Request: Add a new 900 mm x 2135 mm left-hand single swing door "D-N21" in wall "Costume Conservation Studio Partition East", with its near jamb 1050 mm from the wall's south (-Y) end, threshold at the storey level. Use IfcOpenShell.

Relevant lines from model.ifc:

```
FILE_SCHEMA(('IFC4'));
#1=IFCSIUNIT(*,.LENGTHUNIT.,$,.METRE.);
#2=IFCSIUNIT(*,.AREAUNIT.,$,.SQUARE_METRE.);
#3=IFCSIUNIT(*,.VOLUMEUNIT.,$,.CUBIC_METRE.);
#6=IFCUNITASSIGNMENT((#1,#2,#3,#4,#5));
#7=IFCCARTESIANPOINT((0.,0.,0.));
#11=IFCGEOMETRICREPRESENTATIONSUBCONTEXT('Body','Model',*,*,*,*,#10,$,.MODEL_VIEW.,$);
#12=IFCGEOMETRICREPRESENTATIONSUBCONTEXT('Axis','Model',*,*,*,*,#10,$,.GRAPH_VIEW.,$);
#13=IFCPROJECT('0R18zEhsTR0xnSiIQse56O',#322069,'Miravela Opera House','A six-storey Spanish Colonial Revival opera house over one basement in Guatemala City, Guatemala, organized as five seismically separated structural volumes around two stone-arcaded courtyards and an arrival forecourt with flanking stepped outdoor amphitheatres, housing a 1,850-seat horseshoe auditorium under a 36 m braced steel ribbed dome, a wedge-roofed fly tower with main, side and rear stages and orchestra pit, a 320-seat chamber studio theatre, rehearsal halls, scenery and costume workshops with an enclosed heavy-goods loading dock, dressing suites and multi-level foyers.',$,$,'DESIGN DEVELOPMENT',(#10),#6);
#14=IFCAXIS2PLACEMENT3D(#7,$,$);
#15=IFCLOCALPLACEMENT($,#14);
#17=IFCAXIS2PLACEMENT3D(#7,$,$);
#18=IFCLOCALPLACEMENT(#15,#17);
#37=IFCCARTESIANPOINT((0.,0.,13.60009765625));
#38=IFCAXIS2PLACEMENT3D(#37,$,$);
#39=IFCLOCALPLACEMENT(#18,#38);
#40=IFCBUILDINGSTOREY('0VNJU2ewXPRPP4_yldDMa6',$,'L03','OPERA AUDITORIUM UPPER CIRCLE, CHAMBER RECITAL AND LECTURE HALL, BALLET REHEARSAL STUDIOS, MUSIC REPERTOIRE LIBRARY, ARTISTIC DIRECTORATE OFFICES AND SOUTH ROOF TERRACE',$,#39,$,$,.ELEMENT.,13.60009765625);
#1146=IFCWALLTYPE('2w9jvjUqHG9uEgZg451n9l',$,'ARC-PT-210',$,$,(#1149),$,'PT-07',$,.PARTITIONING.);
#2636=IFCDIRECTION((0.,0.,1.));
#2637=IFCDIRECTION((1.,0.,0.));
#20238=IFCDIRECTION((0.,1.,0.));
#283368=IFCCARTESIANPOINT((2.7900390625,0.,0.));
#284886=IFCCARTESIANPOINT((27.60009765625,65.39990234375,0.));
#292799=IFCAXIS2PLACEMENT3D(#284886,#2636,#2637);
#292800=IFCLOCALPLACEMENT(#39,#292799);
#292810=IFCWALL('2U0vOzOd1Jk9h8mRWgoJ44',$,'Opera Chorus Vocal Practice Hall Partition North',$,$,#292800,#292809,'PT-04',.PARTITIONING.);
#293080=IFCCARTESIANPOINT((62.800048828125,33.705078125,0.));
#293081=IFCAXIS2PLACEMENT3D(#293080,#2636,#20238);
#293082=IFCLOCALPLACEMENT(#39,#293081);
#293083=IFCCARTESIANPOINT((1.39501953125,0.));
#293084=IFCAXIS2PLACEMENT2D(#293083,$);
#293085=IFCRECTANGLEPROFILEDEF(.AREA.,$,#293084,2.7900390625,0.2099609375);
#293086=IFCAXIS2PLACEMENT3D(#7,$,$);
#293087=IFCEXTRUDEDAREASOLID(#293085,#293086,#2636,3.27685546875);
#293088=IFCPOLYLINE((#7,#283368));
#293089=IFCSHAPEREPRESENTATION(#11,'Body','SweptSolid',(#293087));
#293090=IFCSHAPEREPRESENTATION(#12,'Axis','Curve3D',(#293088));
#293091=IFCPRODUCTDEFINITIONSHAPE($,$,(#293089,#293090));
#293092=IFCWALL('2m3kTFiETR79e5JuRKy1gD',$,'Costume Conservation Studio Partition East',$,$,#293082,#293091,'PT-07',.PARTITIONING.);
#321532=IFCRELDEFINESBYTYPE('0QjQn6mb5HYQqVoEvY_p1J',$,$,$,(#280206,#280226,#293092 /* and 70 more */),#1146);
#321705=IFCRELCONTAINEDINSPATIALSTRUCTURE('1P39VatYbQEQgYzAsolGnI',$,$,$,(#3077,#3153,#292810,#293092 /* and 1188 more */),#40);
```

```python
import numpy as np
import ifcopenshell
import ifcopenshell.api.feature
import ifcopenshell.api.geometry
import ifcopenshell.api.root
import ifcopenshell.api.spatial
import ifcopenshell.geom
import ifcopenshell.util.element
import ifcopenshell.util.placement
import ifcopenshell.util.representation
import ifcopenshell.util.shape
import ifcopenshell.util.unit

model = ifcopenshell.open("model.ifc")
unit_scale = ifcopenshell.util.unit.calculate_unit_scale(model)
settings = ifcopenshell.geom.settings()


def volume(element):
    """Net volume in cubic metres, openings subtracted."""
    shape = ifcopenshell.geom.create_shape(settings, element)
    return ifcopenshell.util.shape.get_volume(shape.geometry)


wall = model.by_guid("2m3kTFiETR79e5JuRKy1gD")
storey = ifcopenshell.util.element.get_container(wall, ifc_class="IfcBuildingStorey")
context = ifcopenshell.util.representation.get_context(model, "Model", "Body", "MODEL_VIEW")
before = volume(wall)

width, height, from_end, sill = 0.9, 2.135, 1.05, 0.0  # metres

# The wall runs along its own X axis, and the end named is its -X end.
wall_shape = ifcopenshell.geom.create_shape(settings, wall)
x, y, z = ifcopenshell.util.shape.get_vertices(wall_shape.geometry).T
start = x.min() + from_end
face, thickness = float(y.min()), float(y.max() - y.min())
wall_matrix = ifcopenshell.util.placement.get_local_placement(wall.ObjectPlacement)
level = ifcopenshell.util.placement.get_local_placement(storey.ObjectPlacement)[2, 3]


def in_wall(x, y):
    """Placement at x, y metres in the wall's axes, at sill height."""
    matrix = wall_matrix.copy()
    matrix[:, 3] = wall_matrix @ np.array([x / unit_scale, y / unit_scale, 0.0, 1.0])
    matrix[2, 3] = level + sill / unit_scale
    return matrix


# Opening: a box that overshoots both wall faces by 50 mm.
opening = ifcopenshell.api.root.create_entity(model, ifc_class="IfcOpeningElement", predefined_type="OPENING")
box = ifcopenshell.api.geometry.add_wall_representation(
    model, context=context, length=width, height=height, thickness=thickness + 0.1
)
ifcopenshell.api.geometry.assign_representation(model, product=opening, representation=box)
ifcopenshell.api.geometry.edit_object_placement(model, product=opening, matrix=in_wall(start, face - 0.05), is_si=False)
ifcopenshell.api.feature.add_feature(model, feature=opening, element=wall)

door = ifcopenshell.api.root.create_entity(model, ifc_class="IfcDoor", name="D-N21", predefined_type="DOOR")
door.OverallWidth, door.OverallHeight = width / unit_scale, height / unit_scale
door.OperationType = "SINGLE_SWING_LEFT"
body = ifcopenshell.api.geometry.add_door_representation(
    model,
    context=context,
    overall_width=door.OverallWidth,
    overall_height=door.OverallHeight,
    operation_type="SINGLE_SWING_LEFT",
    lining_properties={"LiningDepth": thickness / unit_scale, "ThresholdDepth": thickness / unit_scale},
)
ifcopenshell.api.geometry.assign_representation(model, product=door, representation=body)
ifcopenshell.api.spatial.assign_container(model, products=[door], relating_structure=storey)
ifcopenshell.api.feature.add_filling(model, opening=opening, element=door)

# The lining spans the wall, so the door starts at the wall face.
ifcopenshell.api.geometry.edit_object_placement(model, product=door, matrix=in_wall(start, face), is_si=False)

after = volume(wall)

print(f"wall volume {before:.3f} -> {after:.3f} m3")

model.write("model-out.ifc")
```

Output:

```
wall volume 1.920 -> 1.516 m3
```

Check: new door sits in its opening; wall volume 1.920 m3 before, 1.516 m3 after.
